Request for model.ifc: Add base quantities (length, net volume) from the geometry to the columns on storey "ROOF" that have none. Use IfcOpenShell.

First a look at what the model holds.

```python
import ifcopenshell
import ifcopenshell.util.element
import ifcopenshell.util.unit

model = ifcopenshell.open("model.ifc")
print(model.schema)
for unit_type in ("LENGTHUNIT", "AREAUNIT", "VOLUMEUNIT"):
    print(unit_type, ifcopenshell.util.unit.calculate_unit_scale(model, unit_type))
storey = next(s for s in model.by_type("IfcBuildingStorey") if s.Name == "ROOF")
columns = [e for e in ifcopenshell.util.element.get_decomposition(storey) if e.is_a("IfcColumn")]
for e in sorted(columns, key=lambda e: e.id()):
    print(e.id(), e.is_a(), e.Name, list(ifcopenshell.util.element.get_psets(e, qtos_only=True)), sep=" | ")
```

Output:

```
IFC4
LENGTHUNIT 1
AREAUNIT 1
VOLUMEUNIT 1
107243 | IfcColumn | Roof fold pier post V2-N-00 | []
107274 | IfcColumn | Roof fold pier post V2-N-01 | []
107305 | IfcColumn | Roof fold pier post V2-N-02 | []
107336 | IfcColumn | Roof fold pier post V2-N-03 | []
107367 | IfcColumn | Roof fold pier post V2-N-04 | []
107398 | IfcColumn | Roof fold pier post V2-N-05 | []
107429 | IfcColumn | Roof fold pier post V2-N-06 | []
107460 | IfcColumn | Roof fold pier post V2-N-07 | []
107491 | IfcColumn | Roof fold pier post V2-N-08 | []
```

```python
import ifcopenshell
import ifcopenshell.api.pset
import ifcopenshell.geom
import ifcopenshell.util.element
import ifcopenshell.util.shape
import ifcopenshell.util.unit

model = ifcopenshell.open("model.ifc")
unit_scale = ifcopenshell.util.unit.calculate_unit_scale(model)
volume_scale = ifcopenshell.util.unit.calculate_unit_scale(model, "VOLUMEUNIT")
settings = ifcopenshell.geom.settings()

storey = next(s for s in model.by_type("IfcBuildingStorey") if s.Name == "ROOF")
columns = [e for e in ifcopenshell.util.element.get_decomposition(storey) if e.is_a("IfcColumn")]

for e in sorted(columns, key=lambda e: e.id()):
    if ifcopenshell.util.element.get_psets(e, qtos_only=True, should_inherit=False):
        continue
    # Geometry comes back in metres, in the element's own axes.
    shape = ifcopenshell.geom.create_shape(settings, e)
    values = {
        "Length": ifcopenshell.util.shape.get_z(shape.geometry) / unit_scale,
        "NetVolume": ifcopenshell.util.shape.get_volume(shape.geometry) / volume_scale,
    }
    qto = ifcopenshell.api.pset.add_qto(model, product=e, name="Qto_ColumnBaseQuantities")
    ifcopenshell.api.pset.edit_qto(model, qto=qto, properties=values)
    print(e.id(), {k: round(v, 3) for k, v in values.items()})

model.write("model_updated.ifc")
```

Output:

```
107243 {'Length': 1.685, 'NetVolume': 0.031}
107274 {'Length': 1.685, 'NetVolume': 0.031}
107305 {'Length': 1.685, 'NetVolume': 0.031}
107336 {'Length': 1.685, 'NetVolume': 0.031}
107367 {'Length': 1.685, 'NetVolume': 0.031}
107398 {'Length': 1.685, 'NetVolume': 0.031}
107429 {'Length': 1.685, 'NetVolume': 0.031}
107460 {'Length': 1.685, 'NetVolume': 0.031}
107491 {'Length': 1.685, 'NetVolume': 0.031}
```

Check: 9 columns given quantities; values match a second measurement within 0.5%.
